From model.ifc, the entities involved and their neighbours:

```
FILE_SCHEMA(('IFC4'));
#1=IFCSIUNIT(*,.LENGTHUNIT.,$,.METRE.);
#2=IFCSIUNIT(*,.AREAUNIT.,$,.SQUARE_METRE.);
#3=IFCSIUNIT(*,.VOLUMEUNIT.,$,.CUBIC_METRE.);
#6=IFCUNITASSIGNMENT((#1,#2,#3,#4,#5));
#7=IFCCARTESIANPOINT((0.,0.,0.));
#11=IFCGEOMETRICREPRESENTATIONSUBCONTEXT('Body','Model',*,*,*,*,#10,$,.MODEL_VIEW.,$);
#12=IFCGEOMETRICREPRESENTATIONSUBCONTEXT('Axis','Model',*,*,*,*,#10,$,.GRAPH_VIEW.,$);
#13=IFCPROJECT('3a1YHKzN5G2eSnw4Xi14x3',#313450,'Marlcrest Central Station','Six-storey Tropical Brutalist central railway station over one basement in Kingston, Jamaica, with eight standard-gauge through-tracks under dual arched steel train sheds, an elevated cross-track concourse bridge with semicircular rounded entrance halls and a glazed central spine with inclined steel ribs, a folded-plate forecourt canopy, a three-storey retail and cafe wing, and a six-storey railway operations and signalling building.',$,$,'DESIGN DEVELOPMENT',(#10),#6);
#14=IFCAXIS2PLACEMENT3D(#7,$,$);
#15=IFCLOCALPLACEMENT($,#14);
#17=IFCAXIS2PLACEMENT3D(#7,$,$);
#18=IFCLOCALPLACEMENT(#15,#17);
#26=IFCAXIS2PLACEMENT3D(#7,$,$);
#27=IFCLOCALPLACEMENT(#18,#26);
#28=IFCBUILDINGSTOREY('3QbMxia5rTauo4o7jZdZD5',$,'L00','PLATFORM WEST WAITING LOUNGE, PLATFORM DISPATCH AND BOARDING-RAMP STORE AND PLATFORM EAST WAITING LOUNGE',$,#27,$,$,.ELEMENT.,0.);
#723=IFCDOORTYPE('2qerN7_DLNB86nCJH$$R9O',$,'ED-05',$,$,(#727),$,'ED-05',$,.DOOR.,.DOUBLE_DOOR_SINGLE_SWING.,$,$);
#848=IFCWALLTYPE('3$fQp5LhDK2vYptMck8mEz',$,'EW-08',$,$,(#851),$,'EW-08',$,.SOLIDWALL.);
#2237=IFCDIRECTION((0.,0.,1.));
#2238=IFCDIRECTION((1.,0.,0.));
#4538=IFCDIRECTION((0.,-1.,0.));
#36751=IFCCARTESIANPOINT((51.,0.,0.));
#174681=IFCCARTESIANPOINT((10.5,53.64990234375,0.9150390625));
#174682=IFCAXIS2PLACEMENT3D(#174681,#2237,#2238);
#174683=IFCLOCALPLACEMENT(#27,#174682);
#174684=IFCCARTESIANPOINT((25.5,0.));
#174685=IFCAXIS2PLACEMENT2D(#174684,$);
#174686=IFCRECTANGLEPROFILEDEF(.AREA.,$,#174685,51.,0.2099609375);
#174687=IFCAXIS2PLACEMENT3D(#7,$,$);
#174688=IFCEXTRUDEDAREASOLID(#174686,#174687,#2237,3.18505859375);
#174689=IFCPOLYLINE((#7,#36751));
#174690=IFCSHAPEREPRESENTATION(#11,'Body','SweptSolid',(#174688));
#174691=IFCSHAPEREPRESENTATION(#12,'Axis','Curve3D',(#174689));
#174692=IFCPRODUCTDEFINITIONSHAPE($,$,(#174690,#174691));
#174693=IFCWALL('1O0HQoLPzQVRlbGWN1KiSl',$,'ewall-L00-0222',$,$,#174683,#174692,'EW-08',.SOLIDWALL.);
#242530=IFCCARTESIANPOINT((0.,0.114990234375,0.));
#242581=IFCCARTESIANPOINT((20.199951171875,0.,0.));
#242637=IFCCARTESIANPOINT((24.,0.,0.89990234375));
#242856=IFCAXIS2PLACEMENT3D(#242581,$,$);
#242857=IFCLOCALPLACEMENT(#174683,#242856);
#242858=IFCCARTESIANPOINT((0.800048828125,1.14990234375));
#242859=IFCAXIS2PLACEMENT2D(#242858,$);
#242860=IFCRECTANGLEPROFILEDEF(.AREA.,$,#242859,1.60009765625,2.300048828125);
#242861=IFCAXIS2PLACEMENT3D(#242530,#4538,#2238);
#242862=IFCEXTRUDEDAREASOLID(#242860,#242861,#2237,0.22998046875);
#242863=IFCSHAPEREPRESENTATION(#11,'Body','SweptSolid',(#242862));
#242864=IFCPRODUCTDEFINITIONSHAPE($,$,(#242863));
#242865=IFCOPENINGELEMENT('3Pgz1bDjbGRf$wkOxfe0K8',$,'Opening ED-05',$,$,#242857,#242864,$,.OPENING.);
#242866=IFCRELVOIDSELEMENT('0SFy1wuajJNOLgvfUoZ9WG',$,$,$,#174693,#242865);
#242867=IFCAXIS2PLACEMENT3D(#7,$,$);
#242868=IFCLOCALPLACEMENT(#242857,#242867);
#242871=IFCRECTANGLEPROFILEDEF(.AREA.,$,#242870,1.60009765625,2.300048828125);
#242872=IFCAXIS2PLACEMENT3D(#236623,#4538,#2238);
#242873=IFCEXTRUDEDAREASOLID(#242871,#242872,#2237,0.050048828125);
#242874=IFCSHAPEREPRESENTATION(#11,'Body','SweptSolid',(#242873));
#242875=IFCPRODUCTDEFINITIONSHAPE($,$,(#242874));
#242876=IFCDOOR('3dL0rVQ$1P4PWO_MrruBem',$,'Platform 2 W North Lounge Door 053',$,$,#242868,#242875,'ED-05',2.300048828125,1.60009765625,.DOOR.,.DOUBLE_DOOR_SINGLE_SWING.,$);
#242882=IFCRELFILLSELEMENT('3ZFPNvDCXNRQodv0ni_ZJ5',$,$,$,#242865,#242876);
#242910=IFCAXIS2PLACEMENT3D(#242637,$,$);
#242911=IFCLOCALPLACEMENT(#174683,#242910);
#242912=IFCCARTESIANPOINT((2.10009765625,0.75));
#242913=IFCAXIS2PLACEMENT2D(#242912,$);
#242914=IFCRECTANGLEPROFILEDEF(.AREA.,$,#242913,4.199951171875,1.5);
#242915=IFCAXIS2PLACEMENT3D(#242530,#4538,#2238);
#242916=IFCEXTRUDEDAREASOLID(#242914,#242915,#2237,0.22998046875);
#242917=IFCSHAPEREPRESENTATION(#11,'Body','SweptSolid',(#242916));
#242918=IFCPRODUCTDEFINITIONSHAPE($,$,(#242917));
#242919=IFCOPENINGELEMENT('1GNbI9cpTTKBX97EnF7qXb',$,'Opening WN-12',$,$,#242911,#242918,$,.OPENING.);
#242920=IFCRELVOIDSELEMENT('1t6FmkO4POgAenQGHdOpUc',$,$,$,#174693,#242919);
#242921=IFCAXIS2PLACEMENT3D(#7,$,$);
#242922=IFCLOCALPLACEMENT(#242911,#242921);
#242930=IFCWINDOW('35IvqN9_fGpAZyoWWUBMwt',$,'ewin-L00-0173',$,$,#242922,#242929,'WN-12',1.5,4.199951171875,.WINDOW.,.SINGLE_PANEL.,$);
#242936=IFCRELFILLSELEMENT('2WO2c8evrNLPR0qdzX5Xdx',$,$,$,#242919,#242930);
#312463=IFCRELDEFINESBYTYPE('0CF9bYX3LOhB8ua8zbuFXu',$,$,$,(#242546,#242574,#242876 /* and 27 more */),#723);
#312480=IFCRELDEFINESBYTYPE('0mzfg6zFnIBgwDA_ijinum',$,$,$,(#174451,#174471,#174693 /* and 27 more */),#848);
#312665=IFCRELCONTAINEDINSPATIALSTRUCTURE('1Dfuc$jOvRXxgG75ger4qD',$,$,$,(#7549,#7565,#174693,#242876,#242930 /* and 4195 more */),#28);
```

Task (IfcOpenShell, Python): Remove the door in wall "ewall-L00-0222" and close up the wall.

```python
import ifcopenshell
import ifcopenshell.api.feature
import ifcopenshell.api.root
import ifcopenshell.geom
import ifcopenshell.util.shape

model = ifcopenshell.open("model.ifc")
settings = ifcopenshell.geom.settings()


def volume(element):
    """Net volume in cubic metres, openings subtracted."""
    shape = ifcopenshell.geom.create_shape(settings, element)
    return ifcopenshell.util.shape.get_volume(shape.geometry)


door = model.by_id(242876)
opening = door.FillsVoids[0].RelatingOpeningElement
wall = opening.VoidsElements[0].RelatingBuildingElement
before = volume(wall)

ifcopenshell.api.root.remove_product(model, product=door)
ifcopenshell.api.feature.remove_feature(model, feature=opening)

after = volume(wall)

print(f"wall volume {before:.3f} -> {after:.3f} m3")

model.write("model_rev.ifc")
```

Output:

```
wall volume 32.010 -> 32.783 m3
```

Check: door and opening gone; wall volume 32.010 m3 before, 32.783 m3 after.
